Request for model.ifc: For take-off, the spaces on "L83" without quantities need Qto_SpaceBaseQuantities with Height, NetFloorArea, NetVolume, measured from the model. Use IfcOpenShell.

First a look at what the model holds.

```python
import ifcopenshell
import ifcopenshell.util.element
import ifcopenshell.util.unit

model = ifcopenshell.open("model.ifc")
print(model.schema)
for unit_type in ("LENGTHUNIT", "AREAUNIT", "VOLUMEUNIT"):
    print(unit_type, ifcopenshell.util.unit.calculate_unit_scale(model, unit_type))
storey = next(s for s in model.by_type("IfcBuildingStorey") if s.Name == "L83")
spaces = [e for e in ifcopenshell.util.element.get_decomposition(storey) if e.is_a("IfcSpace")]
for e in sorted(spaces, key=lambda e: e.id()):
    print(e.id(), e.is_a(), e.Name, list(ifcopenshell.util.element.get_psets(e, qtos_only=True)), sep=" | ")
```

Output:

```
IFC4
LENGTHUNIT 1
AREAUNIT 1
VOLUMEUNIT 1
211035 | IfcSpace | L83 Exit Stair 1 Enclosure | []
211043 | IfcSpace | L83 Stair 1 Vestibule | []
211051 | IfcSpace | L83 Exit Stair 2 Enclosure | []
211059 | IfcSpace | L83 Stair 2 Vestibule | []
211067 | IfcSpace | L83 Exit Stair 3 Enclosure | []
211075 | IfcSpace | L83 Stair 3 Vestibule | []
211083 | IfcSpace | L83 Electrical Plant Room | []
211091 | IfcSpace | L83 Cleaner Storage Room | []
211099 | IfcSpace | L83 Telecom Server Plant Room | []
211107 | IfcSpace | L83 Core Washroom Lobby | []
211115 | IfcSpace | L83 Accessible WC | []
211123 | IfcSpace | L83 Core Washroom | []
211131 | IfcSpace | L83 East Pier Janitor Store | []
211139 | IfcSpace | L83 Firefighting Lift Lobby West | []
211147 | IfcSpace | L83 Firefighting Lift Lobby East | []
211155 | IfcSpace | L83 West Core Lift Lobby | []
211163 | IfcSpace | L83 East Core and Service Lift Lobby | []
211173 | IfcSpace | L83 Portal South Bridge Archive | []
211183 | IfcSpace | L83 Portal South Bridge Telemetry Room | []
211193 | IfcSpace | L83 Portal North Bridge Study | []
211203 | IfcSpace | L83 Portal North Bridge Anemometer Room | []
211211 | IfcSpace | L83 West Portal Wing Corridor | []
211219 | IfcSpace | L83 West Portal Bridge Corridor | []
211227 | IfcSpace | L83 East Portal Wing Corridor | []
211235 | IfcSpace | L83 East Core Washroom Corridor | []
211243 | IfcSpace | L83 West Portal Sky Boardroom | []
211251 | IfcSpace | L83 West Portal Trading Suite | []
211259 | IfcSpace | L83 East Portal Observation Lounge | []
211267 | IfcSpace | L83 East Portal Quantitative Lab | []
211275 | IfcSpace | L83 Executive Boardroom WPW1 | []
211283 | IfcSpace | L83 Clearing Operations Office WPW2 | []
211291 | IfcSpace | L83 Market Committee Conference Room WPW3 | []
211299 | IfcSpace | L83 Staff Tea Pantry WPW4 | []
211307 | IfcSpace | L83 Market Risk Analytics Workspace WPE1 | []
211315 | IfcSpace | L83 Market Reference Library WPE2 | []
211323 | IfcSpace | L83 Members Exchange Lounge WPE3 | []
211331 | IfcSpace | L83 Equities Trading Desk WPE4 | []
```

```python
import ifcopenshell
import ifcopenshell.api.pset
import ifcopenshell.geom
import ifcopenshell.util.element
import ifcopenshell.util.shape
import ifcopenshell.util.unit

model = ifcopenshell.open("model.ifc")
unit_scale = ifcopenshell.util.unit.calculate_unit_scale(model)
area_scale = ifcopenshell.util.unit.calculate_unit_scale(model, "AREAUNIT")
volume_scale = ifcopenshell.util.unit.calculate_unit_scale(model, "VOLUMEUNIT")
settings = ifcopenshell.geom.settings()

storey = next(s for s in model.by_type("IfcBuildingStorey") if s.Name == "L83")
spaces = [e for e in ifcopenshell.util.element.get_decomposition(storey) if e.is_a("IfcSpace")]

for e in sorted(spaces, key=lambda e: e.id()):
    if ifcopenshell.util.element.get_psets(e, qtos_only=True, should_inherit=False):
        continue
    # Geometry comes back in metres, in the element's own axes.
    shape = ifcopenshell.geom.create_shape(settings, e)
    values = {
        "Height": ifcopenshell.util.shape.get_z(shape.geometry) / unit_scale,
        "NetFloorArea": ifcopenshell.util.shape.get_footprint_area(shape.geometry) / area_scale,
        "NetVolume": ifcopenshell.util.shape.get_volume(shape.geometry) / volume_scale,
    }
    qto = ifcopenshell.api.pset.add_qto(model, product=e, name="Qto_SpaceBaseQuantities")
    ifcopenshell.api.pset.edit_qto(model, qto=qto, properties=values)
    print(e.id(), {k: round(v, 3) for k, v in values.items()})

model.write("model_rev.ifc")
```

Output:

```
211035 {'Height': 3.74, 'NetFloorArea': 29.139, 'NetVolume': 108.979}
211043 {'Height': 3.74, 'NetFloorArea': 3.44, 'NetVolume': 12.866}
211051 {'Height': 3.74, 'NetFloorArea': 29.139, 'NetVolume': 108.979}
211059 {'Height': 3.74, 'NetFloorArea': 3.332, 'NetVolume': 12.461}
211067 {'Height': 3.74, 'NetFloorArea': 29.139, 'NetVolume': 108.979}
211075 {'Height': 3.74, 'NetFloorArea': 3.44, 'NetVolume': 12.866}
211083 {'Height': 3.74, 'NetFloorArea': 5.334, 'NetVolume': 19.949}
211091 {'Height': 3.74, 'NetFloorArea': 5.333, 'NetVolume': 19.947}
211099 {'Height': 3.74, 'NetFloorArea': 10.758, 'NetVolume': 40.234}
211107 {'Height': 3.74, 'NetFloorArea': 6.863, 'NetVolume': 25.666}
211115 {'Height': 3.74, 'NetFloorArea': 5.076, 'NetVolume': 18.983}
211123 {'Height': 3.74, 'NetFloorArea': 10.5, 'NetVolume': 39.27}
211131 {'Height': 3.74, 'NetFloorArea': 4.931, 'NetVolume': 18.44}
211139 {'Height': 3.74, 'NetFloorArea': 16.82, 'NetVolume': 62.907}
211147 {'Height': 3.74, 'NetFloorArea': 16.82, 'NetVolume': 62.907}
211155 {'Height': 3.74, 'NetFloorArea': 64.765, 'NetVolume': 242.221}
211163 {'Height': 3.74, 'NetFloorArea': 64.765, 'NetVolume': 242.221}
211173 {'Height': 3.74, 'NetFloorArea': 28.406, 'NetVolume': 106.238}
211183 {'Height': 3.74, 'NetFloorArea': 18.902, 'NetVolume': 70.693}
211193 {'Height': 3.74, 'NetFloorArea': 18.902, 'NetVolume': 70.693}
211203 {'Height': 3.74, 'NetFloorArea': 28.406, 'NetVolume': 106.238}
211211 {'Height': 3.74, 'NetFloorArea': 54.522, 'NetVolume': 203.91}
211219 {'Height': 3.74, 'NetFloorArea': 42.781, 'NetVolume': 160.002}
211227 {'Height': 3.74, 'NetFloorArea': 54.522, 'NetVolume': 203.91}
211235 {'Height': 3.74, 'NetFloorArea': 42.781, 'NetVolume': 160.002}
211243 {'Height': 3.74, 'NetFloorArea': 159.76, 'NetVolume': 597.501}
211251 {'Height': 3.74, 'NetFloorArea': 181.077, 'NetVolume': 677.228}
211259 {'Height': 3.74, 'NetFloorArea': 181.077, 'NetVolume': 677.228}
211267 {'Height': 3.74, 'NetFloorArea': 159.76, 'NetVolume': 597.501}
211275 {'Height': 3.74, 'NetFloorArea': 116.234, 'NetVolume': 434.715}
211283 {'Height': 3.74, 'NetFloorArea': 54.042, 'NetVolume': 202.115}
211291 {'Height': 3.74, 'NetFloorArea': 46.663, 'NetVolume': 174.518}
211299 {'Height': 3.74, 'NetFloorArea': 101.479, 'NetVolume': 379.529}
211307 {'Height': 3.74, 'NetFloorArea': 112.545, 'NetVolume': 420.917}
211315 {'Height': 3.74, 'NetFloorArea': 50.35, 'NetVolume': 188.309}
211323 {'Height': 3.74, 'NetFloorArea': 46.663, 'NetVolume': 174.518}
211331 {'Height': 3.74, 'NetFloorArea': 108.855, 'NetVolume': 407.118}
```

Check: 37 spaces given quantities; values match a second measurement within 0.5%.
